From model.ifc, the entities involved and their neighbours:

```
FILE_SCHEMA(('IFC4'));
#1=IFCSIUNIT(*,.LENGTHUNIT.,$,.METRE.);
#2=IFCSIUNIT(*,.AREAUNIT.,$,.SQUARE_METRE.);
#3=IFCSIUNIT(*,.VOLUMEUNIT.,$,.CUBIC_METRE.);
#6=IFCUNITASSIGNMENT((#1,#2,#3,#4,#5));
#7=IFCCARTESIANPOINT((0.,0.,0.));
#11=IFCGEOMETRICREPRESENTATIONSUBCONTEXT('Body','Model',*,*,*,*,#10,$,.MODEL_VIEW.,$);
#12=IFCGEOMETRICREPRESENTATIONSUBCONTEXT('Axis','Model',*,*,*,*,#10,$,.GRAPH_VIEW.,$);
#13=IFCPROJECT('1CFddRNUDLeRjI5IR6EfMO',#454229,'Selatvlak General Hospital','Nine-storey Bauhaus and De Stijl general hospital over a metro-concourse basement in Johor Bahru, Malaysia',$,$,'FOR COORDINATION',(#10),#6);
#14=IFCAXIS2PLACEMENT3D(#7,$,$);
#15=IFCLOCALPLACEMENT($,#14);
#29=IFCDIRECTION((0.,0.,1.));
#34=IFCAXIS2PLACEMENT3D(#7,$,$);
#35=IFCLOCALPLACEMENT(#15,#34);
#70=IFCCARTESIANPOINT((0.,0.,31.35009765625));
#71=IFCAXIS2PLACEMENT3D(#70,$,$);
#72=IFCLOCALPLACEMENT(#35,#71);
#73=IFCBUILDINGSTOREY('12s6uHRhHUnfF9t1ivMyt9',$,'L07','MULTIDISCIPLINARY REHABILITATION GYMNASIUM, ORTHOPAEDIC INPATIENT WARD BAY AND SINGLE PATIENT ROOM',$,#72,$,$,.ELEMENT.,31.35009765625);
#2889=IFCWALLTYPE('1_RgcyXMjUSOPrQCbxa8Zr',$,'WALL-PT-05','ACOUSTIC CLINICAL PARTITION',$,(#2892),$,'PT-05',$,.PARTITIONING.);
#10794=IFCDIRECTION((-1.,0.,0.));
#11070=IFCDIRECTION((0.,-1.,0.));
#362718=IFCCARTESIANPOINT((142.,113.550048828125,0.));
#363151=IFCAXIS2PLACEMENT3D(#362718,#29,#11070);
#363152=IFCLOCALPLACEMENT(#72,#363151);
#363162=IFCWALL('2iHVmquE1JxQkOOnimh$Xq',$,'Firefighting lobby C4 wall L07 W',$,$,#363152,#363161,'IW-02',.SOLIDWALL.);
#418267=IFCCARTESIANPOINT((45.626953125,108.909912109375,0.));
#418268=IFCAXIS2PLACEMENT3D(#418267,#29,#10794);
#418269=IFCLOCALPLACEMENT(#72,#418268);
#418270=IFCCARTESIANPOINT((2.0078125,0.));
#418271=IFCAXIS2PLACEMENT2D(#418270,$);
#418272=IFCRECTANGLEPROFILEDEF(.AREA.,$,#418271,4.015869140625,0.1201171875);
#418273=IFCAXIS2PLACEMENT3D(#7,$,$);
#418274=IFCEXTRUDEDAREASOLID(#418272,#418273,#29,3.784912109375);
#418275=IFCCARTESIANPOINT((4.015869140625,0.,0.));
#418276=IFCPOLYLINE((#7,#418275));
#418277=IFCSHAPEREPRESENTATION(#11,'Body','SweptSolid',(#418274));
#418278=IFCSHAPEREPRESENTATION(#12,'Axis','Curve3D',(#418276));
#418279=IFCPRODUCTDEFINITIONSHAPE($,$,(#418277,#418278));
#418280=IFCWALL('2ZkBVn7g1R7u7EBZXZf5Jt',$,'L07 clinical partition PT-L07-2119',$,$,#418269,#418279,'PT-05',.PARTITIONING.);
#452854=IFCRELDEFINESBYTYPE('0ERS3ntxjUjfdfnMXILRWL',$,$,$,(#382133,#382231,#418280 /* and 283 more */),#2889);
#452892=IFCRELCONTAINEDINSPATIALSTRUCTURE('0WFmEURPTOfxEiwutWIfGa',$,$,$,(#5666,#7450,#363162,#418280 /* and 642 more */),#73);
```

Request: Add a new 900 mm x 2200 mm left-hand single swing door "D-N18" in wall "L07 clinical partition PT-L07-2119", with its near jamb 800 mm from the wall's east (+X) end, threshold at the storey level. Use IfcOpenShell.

```python
import numpy as np
import ifcopenshell
import ifcopenshell.api.feature
import ifcopenshell.api.geometry
import ifcopenshell.api.root
import ifcopenshell.api.spatial
import ifcopenshell.geom
import ifcopenshell.util.element
import ifcopenshell.util.placement
import ifcopenshell.util.representation
import ifcopenshell.util.shape
import ifcopenshell.util.unit

model = ifcopenshell.open("model.ifc")
unit_scale = ifcopenshell.util.unit.calculate_unit_scale(model)
settings = ifcopenshell.geom.settings()


def volume(element):
    """Net volume in cubic metres, openings subtracted."""
    shape = ifcopenshell.geom.create_shape(settings, element)
    return ifcopenshell.util.shape.get_volume(shape.geometry)


wall = model.by_guid("2ZkBVn7g1R7u7EBZXZf5Jt")
storey = ifcopenshell.util.element.get_container(wall, ifc_class="IfcBuildingStorey")
context = ifcopenshell.util.representation.get_context(model, "Model", "Body", "MODEL_VIEW")
before = volume(wall)

width, height, from_end, sill = 0.9, 2.2, 0.8, 0.0  # metres

# The wall runs along its own X axis, and the end named is its -X end.
wall_shape = ifcopenshell.geom.create_shape(settings, wall)
x, y, z = ifcopenshell.util.shape.get_vertices(wall_shape.geometry).T
start = x.min() + from_end
face, thickness = float(y.min()), float(y.max() - y.min())
wall_matrix = ifcopenshell.util.placement.get_local_placement(wall.ObjectPlacement)
level = ifcopenshell.util.placement.get_local_placement(storey.ObjectPlacement)[2, 3]


def in_wall(x, y):
    """Placement at x, y metres in the wall's axes, at sill height."""
    matrix = wall_matrix.copy()
    matrix[:, 3] = wall_matrix @ np.array([x / unit_scale, y / unit_scale, 0.0, 1.0])
    matrix[2, 3] = level + sill / unit_scale
    return matrix


# Opening: a box that overshoots both wall faces by 50 mm.
opening = ifcopenshell.api.root.create_entity(model, ifc_class="IfcOpeningElement", predefined_type="OPENING")
box = ifcopenshell.api.geometry.add_wall_representation(
    model, context=context, length=width, height=height, thickness=thickness + 0.1
)
ifcopenshell.api.geometry.assign_representation(model, product=opening, representation=box)
ifcopenshell.api.geometry.edit_object_placement(model, product=opening, matrix=in_wall(start, face - 0.05), is_si=False)
ifcopenshell.api.feature.add_feature(model, feature=opening, element=wall)

door = ifcopenshell.api.root.create_entity(model, ifc_class="IfcDoor", name="D-N18", predefined_type="DOOR")
door.OverallWidth, door.OverallHeight = width / unit_scale, height / unit_scale
door.OperationType = "SINGLE_SWING_LEFT"
body = ifcopenshell.api.geometry.add_door_representation(
    model,
    context=context,
    overall_width=door.OverallWidth,
    overall_height=door.OverallHeight,
    operation_type="SINGLE_SWING_LEFT",
    lining_properties={"LiningDepth": thickness / unit_scale, "ThresholdDepth": thickness / unit_scale},
)
ifcopenshell.api.geometry.assign_representation(model, product=door, representation=body)
ifcopenshell.api.spatial.assign_container(model, products=[door], relating_structure=storey)
ifcopenshell.api.feature.add_filling(model, opening=opening, element=door)

# The lining spans the wall, so the door starts at the wall face.
ifcopenshell.api.geometry.edit_object_placement(model, product=door, matrix=in_wall(start, face), is_si=False)

after = volume(wall)

print(f"wall volume {before:.3f} -> {after:.3f} m3")

model.write("model_v2.ifc")
```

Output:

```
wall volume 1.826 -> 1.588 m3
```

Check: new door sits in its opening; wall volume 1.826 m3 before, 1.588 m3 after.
